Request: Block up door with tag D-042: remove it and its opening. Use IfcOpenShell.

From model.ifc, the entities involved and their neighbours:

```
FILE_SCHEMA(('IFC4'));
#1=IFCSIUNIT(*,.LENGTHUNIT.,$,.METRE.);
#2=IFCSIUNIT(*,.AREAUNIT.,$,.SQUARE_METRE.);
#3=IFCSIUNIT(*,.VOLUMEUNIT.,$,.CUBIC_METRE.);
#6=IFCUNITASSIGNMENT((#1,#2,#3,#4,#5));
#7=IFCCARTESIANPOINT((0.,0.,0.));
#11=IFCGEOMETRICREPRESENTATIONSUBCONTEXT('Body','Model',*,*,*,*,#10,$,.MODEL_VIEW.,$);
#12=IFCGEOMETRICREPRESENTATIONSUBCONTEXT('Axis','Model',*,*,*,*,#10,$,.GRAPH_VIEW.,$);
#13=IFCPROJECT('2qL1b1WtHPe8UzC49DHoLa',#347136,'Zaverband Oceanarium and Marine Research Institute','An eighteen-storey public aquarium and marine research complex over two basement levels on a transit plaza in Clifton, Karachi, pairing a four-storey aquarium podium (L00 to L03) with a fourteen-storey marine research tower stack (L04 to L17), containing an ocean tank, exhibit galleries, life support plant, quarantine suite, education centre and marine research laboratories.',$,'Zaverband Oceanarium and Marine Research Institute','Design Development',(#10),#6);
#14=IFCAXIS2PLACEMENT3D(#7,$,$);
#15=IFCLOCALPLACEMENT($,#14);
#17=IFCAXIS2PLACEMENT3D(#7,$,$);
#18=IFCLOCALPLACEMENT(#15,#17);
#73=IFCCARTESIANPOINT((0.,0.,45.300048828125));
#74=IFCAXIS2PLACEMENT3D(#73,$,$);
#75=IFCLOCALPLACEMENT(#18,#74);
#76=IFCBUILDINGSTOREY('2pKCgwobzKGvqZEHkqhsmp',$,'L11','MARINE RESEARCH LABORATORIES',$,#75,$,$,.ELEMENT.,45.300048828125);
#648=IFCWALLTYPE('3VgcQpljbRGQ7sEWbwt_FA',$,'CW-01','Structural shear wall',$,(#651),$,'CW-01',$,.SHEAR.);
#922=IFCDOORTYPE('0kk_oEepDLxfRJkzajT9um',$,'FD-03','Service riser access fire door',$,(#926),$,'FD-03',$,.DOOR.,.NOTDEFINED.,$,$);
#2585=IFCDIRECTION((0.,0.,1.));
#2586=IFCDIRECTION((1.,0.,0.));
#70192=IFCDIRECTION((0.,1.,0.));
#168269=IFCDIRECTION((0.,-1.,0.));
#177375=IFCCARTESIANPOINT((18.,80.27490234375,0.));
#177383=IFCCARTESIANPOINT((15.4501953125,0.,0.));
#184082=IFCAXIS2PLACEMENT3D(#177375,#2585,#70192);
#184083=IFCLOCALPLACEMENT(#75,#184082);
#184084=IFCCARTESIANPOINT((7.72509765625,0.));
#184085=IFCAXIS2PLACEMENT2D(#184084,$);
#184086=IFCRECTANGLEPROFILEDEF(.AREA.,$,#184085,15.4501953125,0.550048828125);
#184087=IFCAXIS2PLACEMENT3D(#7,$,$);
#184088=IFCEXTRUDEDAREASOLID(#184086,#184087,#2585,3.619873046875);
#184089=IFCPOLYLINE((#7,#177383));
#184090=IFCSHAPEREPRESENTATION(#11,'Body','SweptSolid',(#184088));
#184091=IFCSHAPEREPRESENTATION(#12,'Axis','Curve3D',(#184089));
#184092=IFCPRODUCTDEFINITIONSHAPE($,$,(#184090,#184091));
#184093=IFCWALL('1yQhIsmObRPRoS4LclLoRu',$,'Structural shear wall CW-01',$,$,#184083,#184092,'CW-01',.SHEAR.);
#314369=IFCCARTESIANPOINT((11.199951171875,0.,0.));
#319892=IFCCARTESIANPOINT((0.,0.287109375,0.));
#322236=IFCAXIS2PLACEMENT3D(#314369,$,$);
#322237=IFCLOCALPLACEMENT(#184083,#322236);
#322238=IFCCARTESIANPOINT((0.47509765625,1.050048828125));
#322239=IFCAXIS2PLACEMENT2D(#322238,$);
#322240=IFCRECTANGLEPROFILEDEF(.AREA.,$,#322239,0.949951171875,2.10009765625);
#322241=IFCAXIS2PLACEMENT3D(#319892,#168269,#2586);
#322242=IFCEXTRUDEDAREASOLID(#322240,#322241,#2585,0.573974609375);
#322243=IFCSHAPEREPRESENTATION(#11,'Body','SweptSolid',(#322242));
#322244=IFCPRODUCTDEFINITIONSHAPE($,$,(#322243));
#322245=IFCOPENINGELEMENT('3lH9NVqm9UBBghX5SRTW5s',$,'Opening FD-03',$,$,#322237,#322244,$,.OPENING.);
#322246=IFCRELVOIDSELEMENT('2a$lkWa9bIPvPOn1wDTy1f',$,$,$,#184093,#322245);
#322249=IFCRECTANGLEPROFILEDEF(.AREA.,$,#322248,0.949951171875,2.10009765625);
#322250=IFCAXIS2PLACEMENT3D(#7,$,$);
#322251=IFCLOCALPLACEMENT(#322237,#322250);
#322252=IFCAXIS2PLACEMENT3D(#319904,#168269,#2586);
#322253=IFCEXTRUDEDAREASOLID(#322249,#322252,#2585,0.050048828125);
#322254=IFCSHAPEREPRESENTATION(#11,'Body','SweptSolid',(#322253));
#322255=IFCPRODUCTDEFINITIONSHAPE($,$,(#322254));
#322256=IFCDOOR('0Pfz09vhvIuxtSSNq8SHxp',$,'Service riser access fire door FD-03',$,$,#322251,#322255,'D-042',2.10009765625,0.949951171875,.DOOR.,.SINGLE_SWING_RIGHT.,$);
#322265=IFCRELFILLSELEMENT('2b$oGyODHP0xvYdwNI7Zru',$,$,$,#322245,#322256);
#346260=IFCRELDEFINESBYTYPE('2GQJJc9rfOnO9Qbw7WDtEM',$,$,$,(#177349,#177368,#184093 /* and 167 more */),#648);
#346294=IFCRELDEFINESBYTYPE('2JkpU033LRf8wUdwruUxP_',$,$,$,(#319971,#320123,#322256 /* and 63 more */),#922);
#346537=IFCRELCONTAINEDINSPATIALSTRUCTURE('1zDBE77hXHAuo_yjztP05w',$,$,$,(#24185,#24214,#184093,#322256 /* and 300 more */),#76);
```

```python
import ifcopenshell
import ifcopenshell.api.feature
import ifcopenshell.api.root
import ifcopenshell.geom
import ifcopenshell.util.shape

model = ifcopenshell.open("model.ifc")
settings = ifcopenshell.geom.settings()


def volume(element):
    """Net volume in cubic metres, openings subtracted."""
    shape = ifcopenshell.geom.create_shape(settings, element)
    return ifcopenshell.util.shape.get_volume(shape.geometry)


door = model.by_id(322256)
opening = door.FillsVoids[0].RelatingOpeningElement
wall = opening.VoidsElements[0].RelatingBuildingElement
before = volume(wall)

ifcopenshell.api.root.remove_product(model, product=door)
ifcopenshell.api.feature.remove_feature(model, feature=opening)

after = volume(wall)

print(f"wall volume {before:.3f} -> {after:.3f} m3")

model.write("model-out.ifc")
```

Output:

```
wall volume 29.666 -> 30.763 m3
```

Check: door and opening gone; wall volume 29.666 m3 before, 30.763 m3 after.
